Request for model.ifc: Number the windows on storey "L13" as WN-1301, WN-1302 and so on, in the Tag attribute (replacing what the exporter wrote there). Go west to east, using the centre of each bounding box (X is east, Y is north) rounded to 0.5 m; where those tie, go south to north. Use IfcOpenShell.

First a look at what the model holds.

```python
import ifcopenshell
import ifcopenshell.util.element
import ifcopenshell.util.placement

model = ifcopenshell.open("model.ifc")
print(model.schema)
storey = next(s for s in model.by_type("IfcBuildingStorey") if s.Name == "L13")
windows = [e for e in ifcopenshell.util.element.get_decomposition(storey) if e.is_a("IfcWindow")]
for e in sorted(windows, key=lambda e: e.id()):
    origin = ifcopenshell.util.placement.get_local_placement(e.ObjectPlacement)[:3, 3]
    print(e.id(), e.Tag, e.Name, origin.round(2) + 0.0, sep=" | ")
```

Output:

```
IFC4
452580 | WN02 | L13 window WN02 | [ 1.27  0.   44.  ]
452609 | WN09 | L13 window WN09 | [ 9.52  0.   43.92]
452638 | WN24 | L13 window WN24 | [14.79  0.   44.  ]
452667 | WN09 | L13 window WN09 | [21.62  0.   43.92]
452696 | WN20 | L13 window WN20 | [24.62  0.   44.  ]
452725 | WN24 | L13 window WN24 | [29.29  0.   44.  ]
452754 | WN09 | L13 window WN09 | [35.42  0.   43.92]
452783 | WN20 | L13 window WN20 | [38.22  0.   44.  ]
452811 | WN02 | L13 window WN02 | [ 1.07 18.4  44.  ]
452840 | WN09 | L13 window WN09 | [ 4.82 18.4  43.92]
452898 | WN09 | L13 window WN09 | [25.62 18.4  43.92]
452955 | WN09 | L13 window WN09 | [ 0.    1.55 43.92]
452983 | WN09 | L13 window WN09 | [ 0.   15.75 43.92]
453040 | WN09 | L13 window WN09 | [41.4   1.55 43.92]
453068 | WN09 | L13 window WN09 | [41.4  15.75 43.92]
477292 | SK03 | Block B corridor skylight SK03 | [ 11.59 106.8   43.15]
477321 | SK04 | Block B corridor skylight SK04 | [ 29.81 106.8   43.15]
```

```python
import ifcopenshell
import ifcopenshell.geom
import ifcopenshell.util.element
import ifcopenshell.util.shape

model = ifcopenshell.open("model.ifc")
settings = ifcopenshell.geom.settings()
settings.set("use-world-coords", True)


def centre(element):
    shape = ifcopenshell.geom.create_shape(settings, element)
    return ifcopenshell.util.shape.get_bbox_centroid(shape.geometry)


storey = next(s for s in model.by_type("IfcBuildingStorey") if s.Name == "L13")
windows = [e for e in ifcopenshell.util.element.get_decomposition(storey) if e.is_a("IfcWindow")]

# Insertion points can sit at a corner or the storey origin, so sort by the geometry (in metres).
centres = {e: centre(e) for e in windows}
windows.sort(key=lambda e: (round(centres[e][0] / 0.5), centres[e][1]))

for i, e in enumerate(windows, start=1):
    number = f"WN-13{i:02d}"
    e.Tag = number
    print(e.id(), number)

model.write("model_v2.ifc")
```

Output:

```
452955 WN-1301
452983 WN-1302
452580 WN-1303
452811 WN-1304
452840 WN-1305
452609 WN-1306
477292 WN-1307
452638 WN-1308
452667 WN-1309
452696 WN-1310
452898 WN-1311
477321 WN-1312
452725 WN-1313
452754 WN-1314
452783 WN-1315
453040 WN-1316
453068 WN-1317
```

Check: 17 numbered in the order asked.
